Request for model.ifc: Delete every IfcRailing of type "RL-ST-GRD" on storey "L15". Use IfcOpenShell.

First a look at what the model holds.

```python
import ifcopenshell
import ifcopenshell.util.element

model = ifcopenshell.open("model.ifc")
print(model.schema)
storey = next(s for s in model.by_type("IfcBuildingStorey") if s.Name == "L15")
railings = [e for e in ifcopenshell.util.element.get_decomposition(storey) if e.is_a("IfcRailing")]
seen = {}
for e in railings:
    element_type = ifcopenshell.util.element.get_type(e)
    name = element_type.Name if element_type not in (None, e) else None
    seen[name] = seen.get(name, 0) + 1
for name, count in sorted(seen.items(), key=str):
    print(count, "x", name)
```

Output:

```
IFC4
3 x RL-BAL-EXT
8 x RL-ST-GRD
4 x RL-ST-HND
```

```python
import ifcopenshell
import ifcopenshell.api.root
import ifcopenshell.util.element

model = ifcopenshell.open("model.ifc")

storey = next(s for s in model.by_type("IfcBuildingStorey") if s.Name == "L15")
railings = [e for e in ifcopenshell.util.element.get_decomposition(storey) if e.is_a("IfcRailing")]
targets = [e for e in railings if (t := ifcopenshell.util.element.get_type(e)) not in (None, e) and t.Name == "RL-ST-GRD"]

for e in targets:
    ifcopenshell.api.root.remove_product(model, product=e)
print(len(targets), "removed")

model.write("model_rev.ifc")
```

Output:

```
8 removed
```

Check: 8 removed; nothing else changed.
